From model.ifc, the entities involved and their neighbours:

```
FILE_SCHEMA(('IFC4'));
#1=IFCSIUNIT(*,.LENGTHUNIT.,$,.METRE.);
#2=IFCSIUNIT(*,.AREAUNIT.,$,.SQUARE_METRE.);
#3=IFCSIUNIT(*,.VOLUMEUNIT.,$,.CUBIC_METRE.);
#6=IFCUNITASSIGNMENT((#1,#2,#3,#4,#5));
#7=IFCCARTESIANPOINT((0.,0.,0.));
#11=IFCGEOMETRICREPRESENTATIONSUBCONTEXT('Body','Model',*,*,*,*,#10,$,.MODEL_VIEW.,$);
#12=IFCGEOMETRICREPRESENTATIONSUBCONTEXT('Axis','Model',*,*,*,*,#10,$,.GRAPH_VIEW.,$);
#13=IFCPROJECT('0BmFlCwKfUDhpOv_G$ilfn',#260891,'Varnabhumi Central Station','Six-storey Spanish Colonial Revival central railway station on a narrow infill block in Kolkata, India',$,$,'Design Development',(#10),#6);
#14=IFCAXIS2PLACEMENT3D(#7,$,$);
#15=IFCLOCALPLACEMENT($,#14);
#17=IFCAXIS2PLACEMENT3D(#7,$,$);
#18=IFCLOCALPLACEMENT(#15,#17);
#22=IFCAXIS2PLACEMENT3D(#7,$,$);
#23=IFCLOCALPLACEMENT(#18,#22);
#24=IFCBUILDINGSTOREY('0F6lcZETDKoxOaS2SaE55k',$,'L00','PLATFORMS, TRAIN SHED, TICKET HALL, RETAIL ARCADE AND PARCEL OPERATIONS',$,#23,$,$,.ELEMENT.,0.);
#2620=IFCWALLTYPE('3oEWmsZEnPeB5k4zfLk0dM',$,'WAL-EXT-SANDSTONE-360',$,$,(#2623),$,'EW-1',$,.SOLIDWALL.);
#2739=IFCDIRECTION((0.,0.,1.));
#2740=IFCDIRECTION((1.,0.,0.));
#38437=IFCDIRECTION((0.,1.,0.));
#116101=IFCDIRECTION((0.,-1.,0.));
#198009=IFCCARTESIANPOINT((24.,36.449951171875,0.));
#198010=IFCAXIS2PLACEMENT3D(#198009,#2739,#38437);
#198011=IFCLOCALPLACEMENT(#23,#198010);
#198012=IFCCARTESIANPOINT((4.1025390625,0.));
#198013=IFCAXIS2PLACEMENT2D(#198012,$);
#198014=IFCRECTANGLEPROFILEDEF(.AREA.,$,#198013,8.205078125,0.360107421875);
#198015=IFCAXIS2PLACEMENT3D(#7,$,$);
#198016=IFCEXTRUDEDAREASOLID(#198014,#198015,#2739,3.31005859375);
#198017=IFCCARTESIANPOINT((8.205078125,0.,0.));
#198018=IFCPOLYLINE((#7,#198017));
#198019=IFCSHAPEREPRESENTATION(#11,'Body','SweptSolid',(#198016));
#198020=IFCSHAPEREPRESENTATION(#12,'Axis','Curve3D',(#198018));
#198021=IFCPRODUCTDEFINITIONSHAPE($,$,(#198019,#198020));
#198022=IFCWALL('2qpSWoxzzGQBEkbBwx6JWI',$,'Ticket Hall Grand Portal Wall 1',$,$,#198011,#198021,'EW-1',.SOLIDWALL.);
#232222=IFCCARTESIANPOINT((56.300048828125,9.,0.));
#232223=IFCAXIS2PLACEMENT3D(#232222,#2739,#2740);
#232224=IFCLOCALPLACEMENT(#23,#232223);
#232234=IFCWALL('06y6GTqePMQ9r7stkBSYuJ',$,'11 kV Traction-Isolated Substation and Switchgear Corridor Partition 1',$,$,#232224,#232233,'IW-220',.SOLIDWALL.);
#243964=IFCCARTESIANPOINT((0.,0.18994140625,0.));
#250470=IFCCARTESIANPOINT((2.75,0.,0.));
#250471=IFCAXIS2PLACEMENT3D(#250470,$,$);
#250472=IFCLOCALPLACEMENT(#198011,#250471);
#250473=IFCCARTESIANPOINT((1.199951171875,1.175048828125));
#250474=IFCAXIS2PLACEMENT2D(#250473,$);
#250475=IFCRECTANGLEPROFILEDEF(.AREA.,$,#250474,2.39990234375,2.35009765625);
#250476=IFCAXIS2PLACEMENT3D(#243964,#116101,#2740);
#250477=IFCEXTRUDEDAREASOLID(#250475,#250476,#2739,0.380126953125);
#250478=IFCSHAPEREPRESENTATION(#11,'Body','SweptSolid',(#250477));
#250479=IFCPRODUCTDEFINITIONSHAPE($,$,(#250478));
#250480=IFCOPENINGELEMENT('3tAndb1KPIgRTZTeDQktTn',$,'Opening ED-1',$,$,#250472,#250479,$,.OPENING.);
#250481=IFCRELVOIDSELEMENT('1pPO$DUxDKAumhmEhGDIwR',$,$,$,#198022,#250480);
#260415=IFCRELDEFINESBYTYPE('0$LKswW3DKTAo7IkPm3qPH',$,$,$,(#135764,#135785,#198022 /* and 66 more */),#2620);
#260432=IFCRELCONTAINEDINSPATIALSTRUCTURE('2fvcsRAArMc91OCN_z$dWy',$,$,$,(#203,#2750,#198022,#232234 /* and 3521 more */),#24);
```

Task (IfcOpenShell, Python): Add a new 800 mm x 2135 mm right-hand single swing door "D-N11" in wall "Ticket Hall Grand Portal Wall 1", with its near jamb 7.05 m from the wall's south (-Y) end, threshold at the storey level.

```python
import numpy as np
import ifcopenshell
import ifcopenshell.api.feature
import ifcopenshell.api.geometry
import ifcopenshell.api.root
import ifcopenshell.api.spatial
import ifcopenshell.geom
import ifcopenshell.util.element
import ifcopenshell.util.placement
import ifcopenshell.util.representation
import ifcopenshell.util.shape
import ifcopenshell.util.unit

model = ifcopenshell.open("model.ifc")
unit_scale = ifcopenshell.util.unit.calculate_unit_scale(model)
settings = ifcopenshell.geom.settings()


def volume(element):
    """Net volume in cubic metres, openings subtracted."""
    shape = ifcopenshell.geom.create_shape(settings, element)
    return ifcopenshell.util.shape.get_volume(shape.geometry)


wall = model.by_guid("2qpSWoxzzGQBEkbBwx6JWI")
storey = ifcopenshell.util.element.get_container(wall, ifc_class="IfcBuildingStorey")
context = ifcopenshell.util.representation.get_context(model, "Model", "Body", "MODEL_VIEW")
before = volume(wall)

width, height, from_end, sill = 0.8, 2.135, 7.05, 0.0  # metres

# The wall runs along its own X axis, and the end named is its -X end.
wall_shape = ifcopenshell.geom.create_shape(settings, wall)
x, y, z = ifcopenshell.util.shape.get_vertices(wall_shape.geometry).T
start = x.min() + from_end
face, thickness = float(y.min()), float(y.max() - y.min())
wall_matrix = ifcopenshell.util.placement.get_local_placement(wall.ObjectPlacement)
level = ifcopenshell.util.placement.get_local_placement(storey.ObjectPlacement)[2, 3]


def in_wall(x, y):
    """Placement at x, y metres in the wall's axes, at sill height."""
    matrix = wall_matrix.copy()
    matrix[:, 3] = wall_matrix @ np.array([x / unit_scale, y / unit_scale, 0.0, 1.0])
    matrix[2, 3] = level + sill / unit_scale
    return matrix


# Opening: a box that overshoots both wall faces by 50 mm.
opening = ifcopenshell.api.root.create_entity(model, ifc_class="IfcOpeningElement", predefined_type="OPENING")
box = ifcopenshell.api.geometry.add_wall_representation(
    model, context=context, length=width, height=height, thickness=thickness + 0.1
)
ifcopenshell.api.geometry.assign_representation(model, product=opening, representation=box)
ifcopenshell.api.geometry.edit_object_placement(model, product=opening, matrix=in_wall(start, face - 0.05), is_si=False)
ifcopenshell.api.feature.add_feature(model, feature=opening, element=wall)

door = ifcopenshell.api.root.create_entity(model, ifc_class="IfcDoor", name="D-N11", predefined_type="DOOR")
door.OverallWidth, door.OverallHeight = width / unit_scale, height / unit_scale
door.OperationType = "SINGLE_SWING_RIGHT"
body = ifcopenshell.api.geometry.add_door_representation(
    model,
    context=context,
    overall_width=door.OverallWidth,
    overall_height=door.OverallHeight,
    operation_type="SINGLE_SWING_RIGHT",
    lining_properties={"LiningDepth": thickness / unit_scale, "ThresholdDepth": thickness / unit_scale},
)
ifcopenshell.api.geometry.assign_representation(model, product=door, representation=body)
ifcopenshell.api.spatial.assign_container(model, products=[door], relating_structure=storey)
ifcopenshell.api.feature.add_filling(model, opening=opening, element=door)

# The lining spans the wall, so the door starts at the wall face.
ifcopenshell.api.geometry.edit_object_placement(model, product=door, matrix=in_wall(start, face), is_si=False)

after = volume(wall)

print(f"wall volume {before:.3f} -> {after:.3f} m3")

model.write("model_v2.ifc")
```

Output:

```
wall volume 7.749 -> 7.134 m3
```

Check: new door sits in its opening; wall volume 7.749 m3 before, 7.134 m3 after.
